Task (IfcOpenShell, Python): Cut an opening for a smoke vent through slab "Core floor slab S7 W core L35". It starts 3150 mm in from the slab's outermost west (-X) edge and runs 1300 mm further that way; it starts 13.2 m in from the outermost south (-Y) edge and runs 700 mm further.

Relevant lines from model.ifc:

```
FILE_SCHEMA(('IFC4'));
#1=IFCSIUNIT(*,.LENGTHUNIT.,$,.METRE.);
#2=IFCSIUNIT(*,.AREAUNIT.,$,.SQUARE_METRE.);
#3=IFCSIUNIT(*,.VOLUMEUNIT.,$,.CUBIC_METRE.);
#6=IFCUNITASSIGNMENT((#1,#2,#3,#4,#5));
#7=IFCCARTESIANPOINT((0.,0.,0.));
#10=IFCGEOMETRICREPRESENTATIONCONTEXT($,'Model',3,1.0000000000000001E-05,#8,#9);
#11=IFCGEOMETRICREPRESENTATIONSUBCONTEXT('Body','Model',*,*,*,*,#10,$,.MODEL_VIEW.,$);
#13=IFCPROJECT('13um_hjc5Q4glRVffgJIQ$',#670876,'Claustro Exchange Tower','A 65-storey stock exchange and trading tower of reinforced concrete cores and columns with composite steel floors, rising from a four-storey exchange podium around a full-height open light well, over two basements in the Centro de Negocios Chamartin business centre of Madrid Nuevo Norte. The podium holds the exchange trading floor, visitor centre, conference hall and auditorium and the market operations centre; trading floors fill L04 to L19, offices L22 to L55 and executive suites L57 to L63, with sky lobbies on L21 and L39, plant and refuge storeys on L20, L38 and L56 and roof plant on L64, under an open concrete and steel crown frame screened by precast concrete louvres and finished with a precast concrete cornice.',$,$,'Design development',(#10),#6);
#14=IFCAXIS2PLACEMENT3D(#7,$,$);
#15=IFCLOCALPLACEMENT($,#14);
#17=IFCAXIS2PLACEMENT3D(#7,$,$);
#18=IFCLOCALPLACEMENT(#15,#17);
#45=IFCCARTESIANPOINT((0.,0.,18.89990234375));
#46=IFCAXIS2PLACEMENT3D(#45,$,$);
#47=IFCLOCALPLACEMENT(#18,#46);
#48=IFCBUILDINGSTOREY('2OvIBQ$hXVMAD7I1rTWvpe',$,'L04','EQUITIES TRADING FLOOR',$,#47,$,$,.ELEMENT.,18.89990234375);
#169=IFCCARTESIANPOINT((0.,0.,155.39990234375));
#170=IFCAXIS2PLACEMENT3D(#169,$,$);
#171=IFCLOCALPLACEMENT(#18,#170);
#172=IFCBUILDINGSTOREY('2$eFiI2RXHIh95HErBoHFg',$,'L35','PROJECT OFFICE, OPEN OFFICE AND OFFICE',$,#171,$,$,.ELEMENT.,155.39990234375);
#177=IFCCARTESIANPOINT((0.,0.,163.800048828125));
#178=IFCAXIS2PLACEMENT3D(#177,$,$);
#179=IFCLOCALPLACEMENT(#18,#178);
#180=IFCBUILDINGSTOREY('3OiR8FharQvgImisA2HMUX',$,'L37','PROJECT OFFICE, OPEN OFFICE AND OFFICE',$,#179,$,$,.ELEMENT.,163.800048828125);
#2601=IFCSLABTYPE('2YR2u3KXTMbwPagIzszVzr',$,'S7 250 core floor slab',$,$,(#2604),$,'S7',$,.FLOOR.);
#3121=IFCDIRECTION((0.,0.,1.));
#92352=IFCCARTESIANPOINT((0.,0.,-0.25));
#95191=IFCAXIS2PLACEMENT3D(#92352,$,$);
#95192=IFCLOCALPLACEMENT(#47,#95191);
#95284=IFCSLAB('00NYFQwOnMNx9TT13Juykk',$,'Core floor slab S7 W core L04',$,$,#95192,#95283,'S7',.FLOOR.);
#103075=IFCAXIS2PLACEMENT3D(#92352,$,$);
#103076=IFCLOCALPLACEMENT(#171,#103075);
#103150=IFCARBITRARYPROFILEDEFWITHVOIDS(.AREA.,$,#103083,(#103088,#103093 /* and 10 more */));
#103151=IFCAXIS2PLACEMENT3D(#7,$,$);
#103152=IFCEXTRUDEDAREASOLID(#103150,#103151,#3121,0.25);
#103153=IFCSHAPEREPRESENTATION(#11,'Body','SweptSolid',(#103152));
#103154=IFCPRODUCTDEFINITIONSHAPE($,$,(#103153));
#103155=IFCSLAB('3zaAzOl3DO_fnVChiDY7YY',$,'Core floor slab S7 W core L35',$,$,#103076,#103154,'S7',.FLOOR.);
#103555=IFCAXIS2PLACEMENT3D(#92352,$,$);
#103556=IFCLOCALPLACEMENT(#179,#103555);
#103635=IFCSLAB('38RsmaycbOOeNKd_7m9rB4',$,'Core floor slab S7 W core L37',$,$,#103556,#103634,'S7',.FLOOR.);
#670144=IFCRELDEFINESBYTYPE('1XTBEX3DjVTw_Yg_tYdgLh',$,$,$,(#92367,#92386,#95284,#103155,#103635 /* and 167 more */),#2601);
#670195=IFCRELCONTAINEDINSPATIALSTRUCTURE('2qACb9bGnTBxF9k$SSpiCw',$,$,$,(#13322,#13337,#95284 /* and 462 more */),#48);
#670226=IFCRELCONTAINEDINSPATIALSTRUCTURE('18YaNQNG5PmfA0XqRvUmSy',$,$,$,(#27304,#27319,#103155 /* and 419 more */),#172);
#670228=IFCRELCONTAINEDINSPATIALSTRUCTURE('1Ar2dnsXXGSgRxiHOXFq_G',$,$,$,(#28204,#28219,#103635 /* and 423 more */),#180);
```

```python
import numpy as np
import ifcopenshell
import ifcopenshell.api.feature
import ifcopenshell.api.geometry
import ifcopenshell.api.root
import ifcopenshell.geom
import ifcopenshell.util.placement
import ifcopenshell.util.representation
import ifcopenshell.util.shape
import ifcopenshell.util.unit

model = ifcopenshell.open("model.ifc")
unit_scale = ifcopenshell.util.unit.calculate_unit_scale(model)
settings = ifcopenshell.geom.settings()


def volume(element):
    """Net volume in cubic metres, openings subtracted."""
    shape = ifcopenshell.geom.create_shape(settings, element)
    return ifcopenshell.util.shape.get_volume(shape.geometry)


slab = model.by_id(103155)
before = volume(slab)

# Extent in the slab's own axes, in metres. The edges named are its -X and -Y sides.
slab_shape = ifcopenshell.geom.create_shape(settings, slab)
vertices = ifcopenshell.util.shape.get_vertices(slab_shape.geometry)
x_min, y_min, bottom = vertices.min(axis=0)
top = vertices[:, 2].max()

opening = ifcopenshell.api.root.create_entity(model, ifc_class="IfcOpeningElement", name="Smoke vent opening", predefined_type="OPENING")
context = ifcopenshell.util.representation.get_context(model, "Model", "Body", "MODEL_VIEW")
width, depth = 1.3, 0.7
outline = [(0.0, 0.0), (width, 0.0), (width, depth), (0.0, depth), (0.0, 0.0)]
# Overshoot both faces by 50 mm so the cut is clean.
shape = ifcopenshell.api.geometry.add_slab_representation(
    model, context=context, depth=top - bottom + 0.1, polyline=outline
)
ifcopenshell.api.geometry.assign_representation(model, product=opening, representation=shape)

matrix = ifcopenshell.util.placement.get_local_placement(slab.ObjectPlacement)
matrix[:, 3] = matrix @ np.append(np.array([x_min + 3.15, y_min + 13.2, bottom - 0.05]) / unit_scale, 1.0)
ifcopenshell.api.geometry.edit_object_placement(model, product=opening, matrix=matrix, is_si=False)
ifcopenshell.api.feature.add_feature(model, feature=opening, element=slab)

after = volume(slab)

print(f"slab volume {before:.3f} -> {after:.3f} m3")

model.write("model-out.ifc")
```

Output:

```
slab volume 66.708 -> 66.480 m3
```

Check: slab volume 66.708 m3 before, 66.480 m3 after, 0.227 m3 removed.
